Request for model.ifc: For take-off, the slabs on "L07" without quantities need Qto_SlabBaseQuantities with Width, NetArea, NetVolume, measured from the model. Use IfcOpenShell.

First a look at what the model holds.

```python
import ifcopenshell
import ifcopenshell.util.element
import ifcopenshell.util.unit

model = ifcopenshell.open("model.ifc")
print(model.schema)
for unit_type in ("LENGTHUNIT", "AREAUNIT", "VOLUMEUNIT"):
    print(unit_type, ifcopenshell.util.unit.calculate_unit_scale(model, unit_type))
storey = next(s for s in model.by_type("IfcBuildingStorey") if s.Name == "L07")
slabs = [e for e in ifcopenshell.util.element.get_decomposition(storey) if e.is_a("IfcSlab")]
for e in sorted(slabs, key=lambda e: e.id()):
    print(e.id(), e.is_a(), e.Name, list(ifcopenshell.util.element.get_psets(e, qtos_only=True)), sep=" | ")
```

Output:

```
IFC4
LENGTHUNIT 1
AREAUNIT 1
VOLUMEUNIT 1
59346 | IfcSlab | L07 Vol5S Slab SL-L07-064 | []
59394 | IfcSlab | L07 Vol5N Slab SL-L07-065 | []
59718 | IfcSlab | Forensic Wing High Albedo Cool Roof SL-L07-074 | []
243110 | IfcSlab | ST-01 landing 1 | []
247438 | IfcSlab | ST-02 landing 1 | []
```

```python
import ifcopenshell
import ifcopenshell.api.pset
import ifcopenshell.geom
import ifcopenshell.util.element
import ifcopenshell.util.shape
import ifcopenshell.util.unit

model = ifcopenshell.open("model.ifc")
unit_scale = ifcopenshell.util.unit.calculate_unit_scale(model)
area_scale = ifcopenshell.util.unit.calculate_unit_scale(model, "AREAUNIT")
volume_scale = ifcopenshell.util.unit.calculate_unit_scale(model, "VOLUMEUNIT")
settings = ifcopenshell.geom.settings()

storey = next(s for s in model.by_type("IfcBuildingStorey") if s.Name == "L07")
slabs = [e for e in ifcopenshell.util.element.get_decomposition(storey) if e.is_a("IfcSlab")]

for e in sorted(slabs, key=lambda e: e.id()):
    if ifcopenshell.util.element.get_psets(e, qtos_only=True, should_inherit=False):
        continue
    # Geometry comes back in metres, in the element's own axes.
    shape = ifcopenshell.geom.create_shape(settings, e)
    values = {
        "Width": ifcopenshell.util.shape.get_z(shape.geometry) / unit_scale,
        "NetArea": ifcopenshell.util.shape.get_footprint_area(shape.geometry) / area_scale,
        "NetVolume": ifcopenshell.util.shape.get_volume(shape.geometry) / volume_scale,
    }
    qto = ifcopenshell.api.pset.add_qto(model, product=e, name="Qto_SlabBaseQuantities")
    ifcopenshell.api.pset.edit_qto(model, qto=qto, properties=values)
    print(e.id(), {k: round(v, 3) for k, v in values.items()})

model.write("model_edited.ifc")
```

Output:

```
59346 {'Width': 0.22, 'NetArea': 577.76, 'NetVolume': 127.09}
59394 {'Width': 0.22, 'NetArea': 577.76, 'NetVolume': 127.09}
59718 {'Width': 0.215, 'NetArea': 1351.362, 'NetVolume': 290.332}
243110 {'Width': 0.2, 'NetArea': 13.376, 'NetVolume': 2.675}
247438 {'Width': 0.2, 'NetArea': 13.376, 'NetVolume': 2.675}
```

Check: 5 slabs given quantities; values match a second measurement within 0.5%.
